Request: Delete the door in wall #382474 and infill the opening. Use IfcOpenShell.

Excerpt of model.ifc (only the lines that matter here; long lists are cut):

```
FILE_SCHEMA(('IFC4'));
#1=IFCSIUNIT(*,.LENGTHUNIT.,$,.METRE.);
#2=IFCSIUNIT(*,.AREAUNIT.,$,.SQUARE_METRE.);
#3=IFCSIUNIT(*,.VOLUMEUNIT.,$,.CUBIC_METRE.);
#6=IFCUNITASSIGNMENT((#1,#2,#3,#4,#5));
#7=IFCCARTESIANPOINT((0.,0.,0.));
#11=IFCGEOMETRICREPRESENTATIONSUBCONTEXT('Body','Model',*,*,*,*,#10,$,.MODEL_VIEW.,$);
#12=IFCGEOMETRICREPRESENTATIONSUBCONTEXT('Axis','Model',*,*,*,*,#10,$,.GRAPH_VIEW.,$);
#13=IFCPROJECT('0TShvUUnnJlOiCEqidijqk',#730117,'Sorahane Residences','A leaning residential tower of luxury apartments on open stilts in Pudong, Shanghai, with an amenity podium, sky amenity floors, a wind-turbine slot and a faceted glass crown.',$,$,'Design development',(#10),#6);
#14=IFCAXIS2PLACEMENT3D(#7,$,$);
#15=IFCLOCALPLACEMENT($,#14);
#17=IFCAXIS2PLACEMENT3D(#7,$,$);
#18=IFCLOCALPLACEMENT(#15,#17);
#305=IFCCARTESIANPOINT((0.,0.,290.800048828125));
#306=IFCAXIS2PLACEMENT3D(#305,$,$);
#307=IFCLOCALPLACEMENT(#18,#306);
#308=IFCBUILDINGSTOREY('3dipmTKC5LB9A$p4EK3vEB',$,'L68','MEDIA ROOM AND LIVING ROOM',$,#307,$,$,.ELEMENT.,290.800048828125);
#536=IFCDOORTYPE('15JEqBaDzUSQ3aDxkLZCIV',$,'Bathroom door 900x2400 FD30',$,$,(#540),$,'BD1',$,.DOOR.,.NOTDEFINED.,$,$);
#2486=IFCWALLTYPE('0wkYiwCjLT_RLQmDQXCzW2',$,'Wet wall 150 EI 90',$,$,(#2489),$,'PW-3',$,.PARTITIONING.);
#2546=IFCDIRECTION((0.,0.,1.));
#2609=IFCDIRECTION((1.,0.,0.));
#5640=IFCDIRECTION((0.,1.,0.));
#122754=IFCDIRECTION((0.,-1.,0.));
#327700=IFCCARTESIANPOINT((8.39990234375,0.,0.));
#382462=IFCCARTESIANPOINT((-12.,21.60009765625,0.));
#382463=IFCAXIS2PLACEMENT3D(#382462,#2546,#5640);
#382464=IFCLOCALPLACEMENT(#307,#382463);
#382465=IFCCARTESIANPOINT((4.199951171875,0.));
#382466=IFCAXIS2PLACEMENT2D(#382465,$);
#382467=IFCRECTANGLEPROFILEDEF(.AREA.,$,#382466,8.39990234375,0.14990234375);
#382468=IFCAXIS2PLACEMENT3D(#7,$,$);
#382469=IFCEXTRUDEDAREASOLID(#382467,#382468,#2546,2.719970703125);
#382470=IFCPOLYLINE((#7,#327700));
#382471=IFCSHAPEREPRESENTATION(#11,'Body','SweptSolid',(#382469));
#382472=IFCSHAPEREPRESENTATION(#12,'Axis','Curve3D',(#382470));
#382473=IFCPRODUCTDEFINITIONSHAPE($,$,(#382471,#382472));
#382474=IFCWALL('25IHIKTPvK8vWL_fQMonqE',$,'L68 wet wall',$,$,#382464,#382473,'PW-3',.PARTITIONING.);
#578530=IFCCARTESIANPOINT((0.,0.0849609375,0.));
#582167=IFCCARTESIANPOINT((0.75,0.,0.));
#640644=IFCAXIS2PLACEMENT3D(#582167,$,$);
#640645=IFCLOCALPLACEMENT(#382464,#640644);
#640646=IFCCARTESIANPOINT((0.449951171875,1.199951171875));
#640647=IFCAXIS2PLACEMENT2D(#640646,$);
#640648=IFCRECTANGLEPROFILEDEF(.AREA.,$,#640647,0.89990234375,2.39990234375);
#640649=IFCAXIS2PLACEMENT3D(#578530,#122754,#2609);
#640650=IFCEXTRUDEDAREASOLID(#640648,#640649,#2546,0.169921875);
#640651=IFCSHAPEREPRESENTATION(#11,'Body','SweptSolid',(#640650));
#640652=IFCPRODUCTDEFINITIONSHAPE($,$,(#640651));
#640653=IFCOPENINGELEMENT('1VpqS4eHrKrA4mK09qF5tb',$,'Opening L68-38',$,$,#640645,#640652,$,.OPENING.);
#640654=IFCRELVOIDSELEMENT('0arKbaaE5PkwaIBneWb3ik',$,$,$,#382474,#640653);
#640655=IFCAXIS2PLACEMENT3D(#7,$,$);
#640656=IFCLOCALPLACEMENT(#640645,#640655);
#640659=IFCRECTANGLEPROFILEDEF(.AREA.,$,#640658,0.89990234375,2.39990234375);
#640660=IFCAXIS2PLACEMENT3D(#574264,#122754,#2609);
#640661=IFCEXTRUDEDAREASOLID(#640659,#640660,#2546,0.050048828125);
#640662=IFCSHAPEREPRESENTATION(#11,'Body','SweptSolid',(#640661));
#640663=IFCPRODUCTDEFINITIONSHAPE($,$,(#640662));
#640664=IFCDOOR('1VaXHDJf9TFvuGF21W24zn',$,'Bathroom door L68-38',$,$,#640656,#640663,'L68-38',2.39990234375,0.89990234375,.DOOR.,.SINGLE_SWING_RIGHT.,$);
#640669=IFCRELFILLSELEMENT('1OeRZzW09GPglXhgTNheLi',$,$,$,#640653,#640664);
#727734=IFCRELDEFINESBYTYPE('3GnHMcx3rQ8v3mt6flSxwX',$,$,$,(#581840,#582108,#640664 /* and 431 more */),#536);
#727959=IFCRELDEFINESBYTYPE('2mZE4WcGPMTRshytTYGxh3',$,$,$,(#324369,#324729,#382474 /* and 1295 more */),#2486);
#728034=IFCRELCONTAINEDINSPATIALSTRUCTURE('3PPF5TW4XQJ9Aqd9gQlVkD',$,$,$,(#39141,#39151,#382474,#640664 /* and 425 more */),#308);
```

```python
import ifcopenshell
import ifcopenshell.api.feature
import ifcopenshell.api.root
import ifcopenshell.geom
import ifcopenshell.util.shape

model = ifcopenshell.open("model.ifc")
settings = ifcopenshell.geom.settings()


def volume(element):
    """Net volume in cubic metres, openings subtracted."""
    shape = ifcopenshell.geom.create_shape(settings, element)
    return ifcopenshell.util.shape.get_volume(shape.geometry)


door = model.by_id(640664)
opening = door.FillsVoids[0].RelatingOpeningElement
wall = opening.VoidsElements[0].RelatingBuildingElement
before = volume(wall)

ifcopenshell.api.root.remove_product(model, product=door)
ifcopenshell.api.feature.remove_feature(model, feature=opening)

after = volume(wall)

print(f"wall volume {before:.3f} -> {after:.3f} m3")

model.write("model_v2.ifc")
```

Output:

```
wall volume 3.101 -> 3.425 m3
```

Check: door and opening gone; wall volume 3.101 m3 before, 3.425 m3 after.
